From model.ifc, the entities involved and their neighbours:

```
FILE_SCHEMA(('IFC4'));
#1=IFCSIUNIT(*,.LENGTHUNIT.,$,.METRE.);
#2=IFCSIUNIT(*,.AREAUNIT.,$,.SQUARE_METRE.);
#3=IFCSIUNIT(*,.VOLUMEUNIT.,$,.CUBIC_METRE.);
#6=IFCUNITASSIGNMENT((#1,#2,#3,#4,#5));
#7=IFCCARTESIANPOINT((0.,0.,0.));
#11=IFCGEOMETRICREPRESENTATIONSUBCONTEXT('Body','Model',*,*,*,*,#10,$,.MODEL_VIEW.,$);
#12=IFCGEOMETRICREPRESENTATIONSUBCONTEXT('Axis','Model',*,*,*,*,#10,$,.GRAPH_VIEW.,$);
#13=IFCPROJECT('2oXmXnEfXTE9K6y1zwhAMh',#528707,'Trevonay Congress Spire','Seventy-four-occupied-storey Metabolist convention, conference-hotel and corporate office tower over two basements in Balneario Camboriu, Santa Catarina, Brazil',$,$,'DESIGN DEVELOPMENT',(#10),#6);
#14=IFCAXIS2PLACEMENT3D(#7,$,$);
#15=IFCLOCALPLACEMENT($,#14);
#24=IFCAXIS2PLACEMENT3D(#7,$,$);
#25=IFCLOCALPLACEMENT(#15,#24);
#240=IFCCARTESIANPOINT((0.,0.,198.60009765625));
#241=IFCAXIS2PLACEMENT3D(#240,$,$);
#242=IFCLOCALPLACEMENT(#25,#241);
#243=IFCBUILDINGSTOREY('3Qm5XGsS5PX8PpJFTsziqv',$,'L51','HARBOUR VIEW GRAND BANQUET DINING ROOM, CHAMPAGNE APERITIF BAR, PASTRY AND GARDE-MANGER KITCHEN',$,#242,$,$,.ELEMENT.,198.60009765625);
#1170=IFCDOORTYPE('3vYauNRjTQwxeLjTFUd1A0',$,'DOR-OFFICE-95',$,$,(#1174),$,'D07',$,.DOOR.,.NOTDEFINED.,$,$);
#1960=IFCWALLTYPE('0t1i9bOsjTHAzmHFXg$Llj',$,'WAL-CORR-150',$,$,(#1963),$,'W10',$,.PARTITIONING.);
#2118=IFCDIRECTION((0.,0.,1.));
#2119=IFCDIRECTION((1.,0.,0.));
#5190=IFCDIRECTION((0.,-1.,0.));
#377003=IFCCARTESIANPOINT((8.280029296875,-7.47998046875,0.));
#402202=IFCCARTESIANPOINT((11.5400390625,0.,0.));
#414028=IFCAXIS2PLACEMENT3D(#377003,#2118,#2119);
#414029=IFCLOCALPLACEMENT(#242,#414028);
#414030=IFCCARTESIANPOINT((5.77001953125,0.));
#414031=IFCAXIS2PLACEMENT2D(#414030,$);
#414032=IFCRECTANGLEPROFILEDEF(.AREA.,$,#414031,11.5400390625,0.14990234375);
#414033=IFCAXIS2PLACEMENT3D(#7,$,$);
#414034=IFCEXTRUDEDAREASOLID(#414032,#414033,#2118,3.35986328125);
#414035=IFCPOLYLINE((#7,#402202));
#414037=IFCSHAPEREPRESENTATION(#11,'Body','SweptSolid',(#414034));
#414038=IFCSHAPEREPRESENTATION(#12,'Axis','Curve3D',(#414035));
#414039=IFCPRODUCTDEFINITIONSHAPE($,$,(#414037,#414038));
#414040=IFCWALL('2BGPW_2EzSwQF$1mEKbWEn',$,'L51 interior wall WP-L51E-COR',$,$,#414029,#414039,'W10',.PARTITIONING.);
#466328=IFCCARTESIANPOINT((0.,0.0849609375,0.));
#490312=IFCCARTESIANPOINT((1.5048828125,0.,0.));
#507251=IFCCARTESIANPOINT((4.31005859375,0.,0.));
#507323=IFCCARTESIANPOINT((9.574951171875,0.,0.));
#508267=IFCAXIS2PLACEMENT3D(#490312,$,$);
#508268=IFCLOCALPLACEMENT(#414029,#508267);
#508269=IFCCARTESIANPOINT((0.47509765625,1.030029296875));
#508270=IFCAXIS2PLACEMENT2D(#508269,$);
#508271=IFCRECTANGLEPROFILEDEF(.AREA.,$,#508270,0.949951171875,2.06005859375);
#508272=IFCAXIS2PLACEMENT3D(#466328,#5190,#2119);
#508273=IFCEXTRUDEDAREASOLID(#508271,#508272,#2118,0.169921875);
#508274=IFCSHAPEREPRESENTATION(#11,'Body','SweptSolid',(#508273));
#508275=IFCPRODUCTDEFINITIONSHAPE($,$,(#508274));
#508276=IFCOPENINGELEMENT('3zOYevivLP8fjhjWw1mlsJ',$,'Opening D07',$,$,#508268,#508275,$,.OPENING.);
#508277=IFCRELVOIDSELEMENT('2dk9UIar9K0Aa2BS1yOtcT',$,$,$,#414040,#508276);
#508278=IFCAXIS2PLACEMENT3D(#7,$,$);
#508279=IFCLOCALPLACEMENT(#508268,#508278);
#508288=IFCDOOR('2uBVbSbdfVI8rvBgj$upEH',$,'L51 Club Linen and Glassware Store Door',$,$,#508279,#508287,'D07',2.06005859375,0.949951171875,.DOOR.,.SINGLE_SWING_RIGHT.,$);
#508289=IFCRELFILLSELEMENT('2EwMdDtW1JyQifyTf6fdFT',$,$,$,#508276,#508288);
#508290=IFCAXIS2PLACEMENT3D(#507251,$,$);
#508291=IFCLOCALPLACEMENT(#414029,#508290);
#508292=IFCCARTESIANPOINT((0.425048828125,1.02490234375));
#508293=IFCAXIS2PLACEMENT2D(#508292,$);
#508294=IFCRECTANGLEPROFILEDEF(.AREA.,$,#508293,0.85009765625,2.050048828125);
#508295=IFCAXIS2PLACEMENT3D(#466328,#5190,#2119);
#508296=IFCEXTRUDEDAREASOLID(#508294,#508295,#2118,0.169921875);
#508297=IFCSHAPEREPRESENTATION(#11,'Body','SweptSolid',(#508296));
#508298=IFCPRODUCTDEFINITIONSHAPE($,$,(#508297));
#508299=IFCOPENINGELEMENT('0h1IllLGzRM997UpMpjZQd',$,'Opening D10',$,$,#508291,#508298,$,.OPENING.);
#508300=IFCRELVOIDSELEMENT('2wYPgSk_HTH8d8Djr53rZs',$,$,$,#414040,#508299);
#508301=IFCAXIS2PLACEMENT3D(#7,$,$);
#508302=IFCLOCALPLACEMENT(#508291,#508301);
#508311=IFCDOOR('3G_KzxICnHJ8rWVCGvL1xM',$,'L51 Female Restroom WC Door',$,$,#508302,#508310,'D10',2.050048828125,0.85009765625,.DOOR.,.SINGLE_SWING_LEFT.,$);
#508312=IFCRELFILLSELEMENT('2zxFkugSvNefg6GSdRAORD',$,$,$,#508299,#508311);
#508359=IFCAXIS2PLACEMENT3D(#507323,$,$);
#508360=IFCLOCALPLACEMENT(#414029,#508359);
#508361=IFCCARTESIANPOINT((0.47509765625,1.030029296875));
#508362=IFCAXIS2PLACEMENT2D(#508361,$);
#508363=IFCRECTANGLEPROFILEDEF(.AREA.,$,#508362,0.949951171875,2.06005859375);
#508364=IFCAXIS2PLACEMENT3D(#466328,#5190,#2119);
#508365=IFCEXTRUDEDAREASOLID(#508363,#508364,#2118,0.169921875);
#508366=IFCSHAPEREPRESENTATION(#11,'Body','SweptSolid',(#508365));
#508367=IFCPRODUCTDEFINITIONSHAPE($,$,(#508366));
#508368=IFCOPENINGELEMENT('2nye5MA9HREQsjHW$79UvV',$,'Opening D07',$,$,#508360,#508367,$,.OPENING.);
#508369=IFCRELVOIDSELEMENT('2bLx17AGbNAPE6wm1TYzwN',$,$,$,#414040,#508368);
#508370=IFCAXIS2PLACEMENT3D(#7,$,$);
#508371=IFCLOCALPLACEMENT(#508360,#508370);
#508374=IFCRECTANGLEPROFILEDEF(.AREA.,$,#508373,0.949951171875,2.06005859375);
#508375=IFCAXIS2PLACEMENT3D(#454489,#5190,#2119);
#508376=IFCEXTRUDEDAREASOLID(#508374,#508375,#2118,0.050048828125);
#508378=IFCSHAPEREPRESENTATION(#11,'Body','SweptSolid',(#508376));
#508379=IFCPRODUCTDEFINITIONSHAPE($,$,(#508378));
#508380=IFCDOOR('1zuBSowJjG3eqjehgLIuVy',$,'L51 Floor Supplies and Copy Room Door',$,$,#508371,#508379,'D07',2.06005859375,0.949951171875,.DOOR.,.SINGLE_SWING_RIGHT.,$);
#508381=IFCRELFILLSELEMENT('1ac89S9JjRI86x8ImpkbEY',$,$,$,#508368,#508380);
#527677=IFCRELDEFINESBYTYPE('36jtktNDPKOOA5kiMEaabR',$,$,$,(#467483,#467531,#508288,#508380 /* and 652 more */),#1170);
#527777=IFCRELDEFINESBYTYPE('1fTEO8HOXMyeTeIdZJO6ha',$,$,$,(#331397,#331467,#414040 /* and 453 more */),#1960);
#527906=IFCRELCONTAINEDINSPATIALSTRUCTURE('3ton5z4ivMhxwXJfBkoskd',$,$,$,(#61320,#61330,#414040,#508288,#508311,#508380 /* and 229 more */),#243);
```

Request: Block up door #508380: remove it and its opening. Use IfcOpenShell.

```python
import ifcopenshell
import ifcopenshell.api.feature
import ifcopenshell.api.root
import ifcopenshell.geom
import ifcopenshell.util.shape

model = ifcopenshell.open("model.ifc")
settings = ifcopenshell.geom.settings()


def volume(element):
    """Net volume in cubic metres, openings subtracted."""
    shape = ifcopenshell.geom.create_shape(settings, element)
    return ifcopenshell.util.shape.get_volume(shape.geometry)


door = model.by_id(508380)
opening = door.FillsVoids[0].RelatingOpeningElement
wall = opening.VoidsElements[0].RelatingBuildingElement
before = volume(wall)

ifcopenshell.api.root.remove_product(model, product=door)
ifcopenshell.api.feature.remove_feature(model, feature=opening)

after = volume(wall)

print(f"wall volume {before:.3f} -> {after:.3f} m3")

model.write("model-out.ifc")
```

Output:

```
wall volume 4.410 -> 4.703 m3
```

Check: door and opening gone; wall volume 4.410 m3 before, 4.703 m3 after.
